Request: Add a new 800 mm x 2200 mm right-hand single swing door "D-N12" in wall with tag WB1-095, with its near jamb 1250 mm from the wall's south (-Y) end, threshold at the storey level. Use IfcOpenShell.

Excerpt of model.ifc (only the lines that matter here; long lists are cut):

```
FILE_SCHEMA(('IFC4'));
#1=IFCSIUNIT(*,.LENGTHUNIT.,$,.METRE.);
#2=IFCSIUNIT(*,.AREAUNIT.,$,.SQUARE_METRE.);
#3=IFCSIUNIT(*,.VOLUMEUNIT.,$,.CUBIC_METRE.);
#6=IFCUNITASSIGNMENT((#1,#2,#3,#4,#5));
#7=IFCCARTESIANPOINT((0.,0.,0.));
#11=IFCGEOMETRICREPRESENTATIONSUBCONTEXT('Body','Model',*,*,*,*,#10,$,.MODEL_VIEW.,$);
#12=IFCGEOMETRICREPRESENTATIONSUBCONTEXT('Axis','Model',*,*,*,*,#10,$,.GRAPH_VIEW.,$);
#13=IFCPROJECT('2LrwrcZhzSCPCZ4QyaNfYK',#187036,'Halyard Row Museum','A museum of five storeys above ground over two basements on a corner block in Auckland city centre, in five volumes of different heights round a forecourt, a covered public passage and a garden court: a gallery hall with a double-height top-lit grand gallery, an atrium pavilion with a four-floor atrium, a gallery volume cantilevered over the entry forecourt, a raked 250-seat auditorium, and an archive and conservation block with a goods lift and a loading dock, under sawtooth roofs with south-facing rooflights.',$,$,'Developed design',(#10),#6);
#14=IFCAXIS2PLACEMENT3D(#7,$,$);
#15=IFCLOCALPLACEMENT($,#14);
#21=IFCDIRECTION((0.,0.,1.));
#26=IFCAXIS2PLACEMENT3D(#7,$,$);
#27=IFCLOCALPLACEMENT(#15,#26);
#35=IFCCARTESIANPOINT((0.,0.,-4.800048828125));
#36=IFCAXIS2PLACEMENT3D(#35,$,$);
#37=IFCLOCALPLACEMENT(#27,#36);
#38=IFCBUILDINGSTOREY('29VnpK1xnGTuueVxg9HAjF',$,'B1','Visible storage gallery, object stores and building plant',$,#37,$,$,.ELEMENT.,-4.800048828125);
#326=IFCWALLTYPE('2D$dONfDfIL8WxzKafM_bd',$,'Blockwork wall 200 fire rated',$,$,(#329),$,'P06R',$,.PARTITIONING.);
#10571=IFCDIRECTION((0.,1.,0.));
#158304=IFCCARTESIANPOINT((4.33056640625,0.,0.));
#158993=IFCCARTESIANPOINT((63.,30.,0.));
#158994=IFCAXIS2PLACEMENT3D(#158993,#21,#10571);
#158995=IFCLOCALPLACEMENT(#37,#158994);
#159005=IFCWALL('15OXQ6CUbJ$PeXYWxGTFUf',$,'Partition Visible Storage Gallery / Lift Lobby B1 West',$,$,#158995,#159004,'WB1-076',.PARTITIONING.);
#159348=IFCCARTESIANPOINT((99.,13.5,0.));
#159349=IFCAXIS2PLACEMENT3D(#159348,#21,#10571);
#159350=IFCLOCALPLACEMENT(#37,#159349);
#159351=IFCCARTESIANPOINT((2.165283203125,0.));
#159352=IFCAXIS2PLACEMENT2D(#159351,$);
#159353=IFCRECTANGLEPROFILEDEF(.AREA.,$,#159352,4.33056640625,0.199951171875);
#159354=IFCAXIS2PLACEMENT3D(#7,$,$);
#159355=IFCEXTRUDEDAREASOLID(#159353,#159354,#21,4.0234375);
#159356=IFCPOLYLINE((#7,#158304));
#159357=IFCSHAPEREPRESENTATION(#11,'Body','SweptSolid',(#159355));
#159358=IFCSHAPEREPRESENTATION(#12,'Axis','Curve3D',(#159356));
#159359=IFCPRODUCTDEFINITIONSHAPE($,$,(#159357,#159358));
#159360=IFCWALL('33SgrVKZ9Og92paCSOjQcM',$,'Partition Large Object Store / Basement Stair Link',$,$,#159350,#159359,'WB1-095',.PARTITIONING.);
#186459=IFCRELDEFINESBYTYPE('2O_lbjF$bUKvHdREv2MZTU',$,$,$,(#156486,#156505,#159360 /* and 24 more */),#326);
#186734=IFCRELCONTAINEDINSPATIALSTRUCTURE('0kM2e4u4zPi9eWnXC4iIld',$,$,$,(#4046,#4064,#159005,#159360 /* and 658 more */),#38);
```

```python
import numpy as np
import ifcopenshell
import ifcopenshell.api.feature
import ifcopenshell.api.geometry
import ifcopenshell.api.root
import ifcopenshell.api.spatial
import ifcopenshell.geom
import ifcopenshell.util.element
import ifcopenshell.util.placement
import ifcopenshell.util.representation
import ifcopenshell.util.shape
import ifcopenshell.util.unit

model = ifcopenshell.open("model.ifc")
unit_scale = ifcopenshell.util.unit.calculate_unit_scale(model)
settings = ifcopenshell.geom.settings()


def volume(element):
    """Net volume in cubic metres, openings subtracted."""
    shape = ifcopenshell.geom.create_shape(settings, element)
    return ifcopenshell.util.shape.get_volume(shape.geometry)


wall = model.by_guid("33SgrVKZ9Og92paCSOjQcM")
storey = ifcopenshell.util.element.get_container(wall, ifc_class="IfcBuildingStorey")
context = ifcopenshell.util.representation.get_context(model, "Model", "Body", "MODEL_VIEW")
before = volume(wall)

width, height, from_end, sill = 0.8, 2.2, 1.25, 0.0  # metres

# The wall runs along its own X axis, and the end named is its -X end.
wall_shape = ifcopenshell.geom.create_shape(settings, wall)
x, y, z = ifcopenshell.util.shape.get_vertices(wall_shape.geometry).T
start = x.min() + from_end
face, thickness = float(y.min()), float(y.max() - y.min())
wall_matrix = ifcopenshell.util.placement.get_local_placement(wall.ObjectPlacement)
level = ifcopenshell.util.placement.get_local_placement(storey.ObjectPlacement)[2, 3]


def in_wall(x, y):
    """Placement at x, y metres in the wall's axes, at sill height."""
    matrix = wall_matrix.copy()
    matrix[:, 3] = wall_matrix @ np.array([x / unit_scale, y / unit_scale, 0.0, 1.0])
    matrix[2, 3] = level + sill / unit_scale
    return matrix


# Opening: a box that overshoots both wall faces by 50 mm.
opening = ifcopenshell.api.root.create_entity(model, ifc_class="IfcOpeningElement", predefined_type="OPENING")
box = ifcopenshell.api.geometry.add_wall_representation(
    model, context=context, length=width, height=height, thickness=thickness + 0.1
)
ifcopenshell.api.geometry.assign_representation(model, product=opening, representation=box)
ifcopenshell.api.geometry.edit_object_placement(model, product=opening, matrix=in_wall(start, face - 0.05), is_si=False)
ifcopenshell.api.feature.add_feature(model, feature=opening, element=wall)

door = ifcopenshell.api.root.create_entity(model, ifc_class="IfcDoor", name="D-N12", predefined_type="DOOR")
door.OverallWidth, door.OverallHeight = width / unit_scale, height / unit_scale
door.OperationType = "SINGLE_SWING_RIGHT"
body = ifcopenshell.api.geometry.add_door_representation(
    model,
    context=context,
    overall_width=door.OverallWidth,
    overall_height=door.OverallHeight,
    operation_type="SINGLE_SWING_RIGHT",
    lining_properties={"LiningDepth": thickness / unit_scale, "ThresholdDepth": thickness / unit_scale},
)
ifcopenshell.api.geometry.assign_representation(model, product=door, representation=body)
ifcopenshell.api.spatial.assign_container(model, products=[door], relating_structure=storey)
ifcopenshell.api.feature.add_filling(model, opening=opening, element=door)

# The lining spans the wall, so the door starts at the wall face.
ifcopenshell.api.geometry.edit_object_placement(model, product=door, matrix=in_wall(start, face), is_si=False)

after = volume(wall)

print(f"wall volume {before:.3f} -> {after:.3f} m3")

model.write("model_rev.ifc")
```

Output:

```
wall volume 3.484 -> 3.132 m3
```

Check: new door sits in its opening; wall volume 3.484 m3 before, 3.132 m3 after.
